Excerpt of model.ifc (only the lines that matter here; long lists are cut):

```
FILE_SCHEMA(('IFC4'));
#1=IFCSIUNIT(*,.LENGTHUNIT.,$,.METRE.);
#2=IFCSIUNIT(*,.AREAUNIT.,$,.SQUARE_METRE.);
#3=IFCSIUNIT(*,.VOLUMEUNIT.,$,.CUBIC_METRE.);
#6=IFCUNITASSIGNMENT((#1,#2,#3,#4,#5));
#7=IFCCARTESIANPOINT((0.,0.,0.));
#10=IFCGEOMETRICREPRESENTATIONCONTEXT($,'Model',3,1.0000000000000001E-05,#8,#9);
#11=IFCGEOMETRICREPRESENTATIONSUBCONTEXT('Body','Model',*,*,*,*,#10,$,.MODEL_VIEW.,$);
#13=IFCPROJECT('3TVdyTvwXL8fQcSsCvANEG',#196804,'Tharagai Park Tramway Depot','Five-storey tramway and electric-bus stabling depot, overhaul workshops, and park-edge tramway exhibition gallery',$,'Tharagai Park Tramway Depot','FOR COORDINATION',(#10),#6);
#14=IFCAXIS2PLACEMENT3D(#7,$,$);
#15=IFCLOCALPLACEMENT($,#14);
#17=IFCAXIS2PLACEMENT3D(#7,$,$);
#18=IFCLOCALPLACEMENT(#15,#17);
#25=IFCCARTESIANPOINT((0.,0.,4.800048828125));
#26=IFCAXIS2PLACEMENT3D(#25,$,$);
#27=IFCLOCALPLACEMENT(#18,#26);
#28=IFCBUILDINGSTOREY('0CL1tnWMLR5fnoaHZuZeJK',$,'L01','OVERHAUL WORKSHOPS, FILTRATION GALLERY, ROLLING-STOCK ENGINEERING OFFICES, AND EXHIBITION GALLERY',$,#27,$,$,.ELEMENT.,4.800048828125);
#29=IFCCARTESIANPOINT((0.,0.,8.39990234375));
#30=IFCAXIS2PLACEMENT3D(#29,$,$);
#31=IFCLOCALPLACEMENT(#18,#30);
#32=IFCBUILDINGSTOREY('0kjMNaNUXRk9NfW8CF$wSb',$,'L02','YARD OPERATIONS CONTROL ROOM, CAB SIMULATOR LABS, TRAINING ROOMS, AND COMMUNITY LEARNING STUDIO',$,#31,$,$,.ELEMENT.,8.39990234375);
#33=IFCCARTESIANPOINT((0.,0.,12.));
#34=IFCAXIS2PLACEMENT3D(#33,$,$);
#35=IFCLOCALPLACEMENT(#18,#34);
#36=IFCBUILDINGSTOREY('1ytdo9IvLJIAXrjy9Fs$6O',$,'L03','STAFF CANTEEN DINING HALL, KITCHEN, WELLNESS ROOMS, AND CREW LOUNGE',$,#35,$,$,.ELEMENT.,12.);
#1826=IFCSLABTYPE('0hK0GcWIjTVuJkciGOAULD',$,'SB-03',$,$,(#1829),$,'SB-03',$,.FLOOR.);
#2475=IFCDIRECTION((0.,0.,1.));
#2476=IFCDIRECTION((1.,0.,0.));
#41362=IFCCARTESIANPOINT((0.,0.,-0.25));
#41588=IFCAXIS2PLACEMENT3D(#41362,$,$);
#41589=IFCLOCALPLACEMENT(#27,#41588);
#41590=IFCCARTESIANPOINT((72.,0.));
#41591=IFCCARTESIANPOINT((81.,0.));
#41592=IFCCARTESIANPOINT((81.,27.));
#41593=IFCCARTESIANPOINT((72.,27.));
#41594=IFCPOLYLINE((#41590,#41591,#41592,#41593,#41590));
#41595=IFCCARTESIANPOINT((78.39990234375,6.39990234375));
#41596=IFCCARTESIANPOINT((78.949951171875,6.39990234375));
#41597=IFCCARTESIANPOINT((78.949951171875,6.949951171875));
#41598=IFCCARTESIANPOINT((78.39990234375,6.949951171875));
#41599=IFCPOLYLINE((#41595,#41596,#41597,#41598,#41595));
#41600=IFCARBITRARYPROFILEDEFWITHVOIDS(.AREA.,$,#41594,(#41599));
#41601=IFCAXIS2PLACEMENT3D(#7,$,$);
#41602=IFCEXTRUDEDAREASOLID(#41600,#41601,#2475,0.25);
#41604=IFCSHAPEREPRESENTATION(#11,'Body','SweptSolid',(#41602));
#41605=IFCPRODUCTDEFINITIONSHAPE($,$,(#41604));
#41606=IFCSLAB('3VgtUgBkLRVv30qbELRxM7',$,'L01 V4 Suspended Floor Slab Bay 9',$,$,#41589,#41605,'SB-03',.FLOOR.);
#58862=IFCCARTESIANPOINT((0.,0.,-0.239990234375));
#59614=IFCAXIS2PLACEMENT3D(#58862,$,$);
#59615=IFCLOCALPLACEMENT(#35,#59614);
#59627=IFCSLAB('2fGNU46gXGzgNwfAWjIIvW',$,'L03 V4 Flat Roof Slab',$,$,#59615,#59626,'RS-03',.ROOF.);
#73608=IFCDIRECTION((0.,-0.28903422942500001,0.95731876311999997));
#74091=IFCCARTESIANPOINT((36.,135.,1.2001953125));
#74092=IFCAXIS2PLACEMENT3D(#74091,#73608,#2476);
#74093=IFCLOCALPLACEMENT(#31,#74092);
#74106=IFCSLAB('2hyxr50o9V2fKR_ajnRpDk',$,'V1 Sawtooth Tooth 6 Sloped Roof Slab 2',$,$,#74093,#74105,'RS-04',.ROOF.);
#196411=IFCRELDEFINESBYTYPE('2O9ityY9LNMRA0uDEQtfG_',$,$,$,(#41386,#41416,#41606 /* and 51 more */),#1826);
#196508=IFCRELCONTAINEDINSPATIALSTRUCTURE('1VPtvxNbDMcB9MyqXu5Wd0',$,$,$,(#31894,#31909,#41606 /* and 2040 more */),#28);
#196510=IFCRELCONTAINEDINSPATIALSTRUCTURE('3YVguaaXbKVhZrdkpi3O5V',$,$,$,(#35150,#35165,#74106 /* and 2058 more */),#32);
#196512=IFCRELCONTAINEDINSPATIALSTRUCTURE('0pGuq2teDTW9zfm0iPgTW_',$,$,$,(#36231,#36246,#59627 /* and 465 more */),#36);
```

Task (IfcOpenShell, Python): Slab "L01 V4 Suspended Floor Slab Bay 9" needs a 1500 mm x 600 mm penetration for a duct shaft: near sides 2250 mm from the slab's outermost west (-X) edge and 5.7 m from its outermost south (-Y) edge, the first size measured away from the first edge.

```python
import numpy as np
import ifcopenshell
import ifcopenshell.api.feature
import ifcopenshell.api.geometry
import ifcopenshell.api.root
import ifcopenshell.geom
import ifcopenshell.util.placement
import ifcopenshell.util.representation
import ifcopenshell.util.shape
import ifcopenshell.util.unit

model = ifcopenshell.open("model.ifc")
unit_scale = ifcopenshell.util.unit.calculate_unit_scale(model)
settings = ifcopenshell.geom.settings()


def volume(element):
    """Net volume in cubic metres, openings subtracted."""
    shape = ifcopenshell.geom.create_shape(settings, element)
    return ifcopenshell.util.shape.get_volume(shape.geometry)


slab = model.by_guid("3VgtUgBkLRVv30qbELRxM7")
before = volume(slab)

# Extent in the slab's own axes, in metres. The edges named are its -X and -Y sides.
slab_shape = ifcopenshell.geom.create_shape(settings, slab)
vertices = ifcopenshell.util.shape.get_vertices(slab_shape.geometry)
x_min, y_min, bottom = vertices.min(axis=0)
top = vertices[:, 2].max()

opening = ifcopenshell.api.root.create_entity(model, ifc_class="IfcOpeningElement", name="Duct shaft opening", predefined_type="OPENING")
context = ifcopenshell.util.representation.get_context(model, "Model", "Body", "MODEL_VIEW")
width, depth = 1.5, 0.6
outline = [(0.0, 0.0), (width, 0.0), (width, depth), (0.0, depth), (0.0, 0.0)]
# Overshoot both faces by 50 mm so the cut is clean.
shape = ifcopenshell.api.geometry.add_slab_representation(
    model, context=context, depth=top - bottom + 0.1, polyline=outline
)
ifcopenshell.api.geometry.assign_representation(model, product=opening, representation=shape)

matrix = ifcopenshell.util.placement.get_local_placement(slab.ObjectPlacement)
matrix[:, 3] = matrix @ np.append(np.array([x_min + 2.25, y_min + 5.7, bottom - 0.05]) / unit_scale, 1.0)
ifcopenshell.api.geometry.edit_object_placement(model, product=opening, matrix=matrix, is_si=False)
ifcopenshell.api.feature.add_feature(model, feature=opening, element=slab)

after = volume(slab)

print(f"slab volume {before:.3f} -> {after:.3f} m3")

model.write("model-out.ifc")
```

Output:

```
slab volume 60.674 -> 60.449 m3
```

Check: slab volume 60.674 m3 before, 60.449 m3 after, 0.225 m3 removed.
